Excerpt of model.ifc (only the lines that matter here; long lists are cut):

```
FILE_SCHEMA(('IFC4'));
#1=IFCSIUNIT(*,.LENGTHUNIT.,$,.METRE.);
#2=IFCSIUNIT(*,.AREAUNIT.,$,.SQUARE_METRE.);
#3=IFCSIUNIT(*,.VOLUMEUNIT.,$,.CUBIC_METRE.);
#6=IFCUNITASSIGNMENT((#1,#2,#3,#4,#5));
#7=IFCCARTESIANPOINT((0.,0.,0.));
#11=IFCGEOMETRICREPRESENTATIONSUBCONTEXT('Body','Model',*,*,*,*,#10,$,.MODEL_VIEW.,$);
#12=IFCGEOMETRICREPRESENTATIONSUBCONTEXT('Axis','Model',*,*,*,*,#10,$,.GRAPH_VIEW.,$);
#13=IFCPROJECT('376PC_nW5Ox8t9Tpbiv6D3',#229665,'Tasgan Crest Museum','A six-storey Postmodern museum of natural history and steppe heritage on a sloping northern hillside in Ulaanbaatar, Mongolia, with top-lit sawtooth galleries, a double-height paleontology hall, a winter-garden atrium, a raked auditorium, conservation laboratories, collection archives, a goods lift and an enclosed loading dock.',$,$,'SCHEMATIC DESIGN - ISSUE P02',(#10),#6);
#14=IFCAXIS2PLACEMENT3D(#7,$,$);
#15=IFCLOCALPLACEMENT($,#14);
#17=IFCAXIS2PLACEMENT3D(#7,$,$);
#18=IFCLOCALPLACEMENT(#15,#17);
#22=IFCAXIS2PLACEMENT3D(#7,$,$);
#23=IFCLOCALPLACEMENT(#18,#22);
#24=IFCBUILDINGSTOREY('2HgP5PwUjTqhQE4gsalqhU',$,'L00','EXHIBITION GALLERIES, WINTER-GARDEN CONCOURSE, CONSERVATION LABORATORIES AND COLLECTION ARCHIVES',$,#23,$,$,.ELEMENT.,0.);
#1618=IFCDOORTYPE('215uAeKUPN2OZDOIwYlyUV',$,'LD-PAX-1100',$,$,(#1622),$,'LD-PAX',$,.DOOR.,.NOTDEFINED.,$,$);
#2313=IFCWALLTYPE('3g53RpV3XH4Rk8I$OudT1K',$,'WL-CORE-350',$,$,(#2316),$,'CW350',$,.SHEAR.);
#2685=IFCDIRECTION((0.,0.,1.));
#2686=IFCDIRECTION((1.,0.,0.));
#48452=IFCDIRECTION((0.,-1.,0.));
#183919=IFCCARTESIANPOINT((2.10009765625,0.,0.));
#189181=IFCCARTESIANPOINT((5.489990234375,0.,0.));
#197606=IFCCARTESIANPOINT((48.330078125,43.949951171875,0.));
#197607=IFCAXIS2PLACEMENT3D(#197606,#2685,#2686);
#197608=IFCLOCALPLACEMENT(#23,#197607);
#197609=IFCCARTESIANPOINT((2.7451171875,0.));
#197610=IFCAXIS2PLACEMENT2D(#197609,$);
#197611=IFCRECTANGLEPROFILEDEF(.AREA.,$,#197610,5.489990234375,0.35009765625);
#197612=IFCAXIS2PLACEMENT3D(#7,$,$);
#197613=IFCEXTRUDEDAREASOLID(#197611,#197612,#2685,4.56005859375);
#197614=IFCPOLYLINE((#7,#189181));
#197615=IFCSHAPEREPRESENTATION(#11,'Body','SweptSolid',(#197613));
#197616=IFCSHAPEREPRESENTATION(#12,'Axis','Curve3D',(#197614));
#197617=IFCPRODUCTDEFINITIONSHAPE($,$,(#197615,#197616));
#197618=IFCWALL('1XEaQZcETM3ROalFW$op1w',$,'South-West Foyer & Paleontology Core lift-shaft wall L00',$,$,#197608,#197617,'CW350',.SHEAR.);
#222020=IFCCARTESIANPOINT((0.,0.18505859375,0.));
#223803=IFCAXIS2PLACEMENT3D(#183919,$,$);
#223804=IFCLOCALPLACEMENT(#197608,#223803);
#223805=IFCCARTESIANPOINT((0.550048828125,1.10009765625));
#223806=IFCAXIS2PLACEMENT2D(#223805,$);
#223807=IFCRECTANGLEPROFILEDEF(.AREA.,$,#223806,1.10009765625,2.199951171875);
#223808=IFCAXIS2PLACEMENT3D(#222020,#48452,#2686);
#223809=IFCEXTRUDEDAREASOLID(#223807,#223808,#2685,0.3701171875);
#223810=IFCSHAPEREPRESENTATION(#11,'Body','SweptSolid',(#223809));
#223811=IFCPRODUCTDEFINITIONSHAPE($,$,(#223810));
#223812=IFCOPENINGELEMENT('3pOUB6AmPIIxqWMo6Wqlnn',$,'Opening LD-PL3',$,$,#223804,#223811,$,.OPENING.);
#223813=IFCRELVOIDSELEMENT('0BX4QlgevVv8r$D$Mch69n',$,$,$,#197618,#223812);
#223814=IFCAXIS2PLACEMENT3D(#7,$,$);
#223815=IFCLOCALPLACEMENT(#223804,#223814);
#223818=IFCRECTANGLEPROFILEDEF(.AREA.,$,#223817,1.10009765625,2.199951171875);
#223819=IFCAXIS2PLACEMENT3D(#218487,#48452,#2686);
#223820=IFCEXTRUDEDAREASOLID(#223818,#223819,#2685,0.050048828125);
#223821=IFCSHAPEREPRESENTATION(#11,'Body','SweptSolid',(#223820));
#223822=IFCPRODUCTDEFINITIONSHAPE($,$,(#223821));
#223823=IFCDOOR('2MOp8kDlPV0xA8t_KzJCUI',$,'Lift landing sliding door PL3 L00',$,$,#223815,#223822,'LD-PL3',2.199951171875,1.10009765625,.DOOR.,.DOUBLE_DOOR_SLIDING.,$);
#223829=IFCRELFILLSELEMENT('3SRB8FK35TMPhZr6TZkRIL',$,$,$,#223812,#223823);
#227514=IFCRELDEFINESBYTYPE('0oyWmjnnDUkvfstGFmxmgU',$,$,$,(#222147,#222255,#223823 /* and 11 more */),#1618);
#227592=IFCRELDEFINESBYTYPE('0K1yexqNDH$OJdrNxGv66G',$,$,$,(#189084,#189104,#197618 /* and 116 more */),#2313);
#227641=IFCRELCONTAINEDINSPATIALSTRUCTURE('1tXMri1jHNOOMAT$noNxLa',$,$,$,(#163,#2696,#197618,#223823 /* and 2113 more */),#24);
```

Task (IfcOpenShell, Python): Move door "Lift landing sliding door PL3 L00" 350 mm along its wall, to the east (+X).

```python
import ifcopenshell
import ifcopenshell.api.geometry
import ifcopenshell.util.placement

model = ifcopenshell.open("model.ifc")

door = model.by_guid("2MOp8kDlPV0xA8t_KzJCUI")
opening = door.FillsVoids[0].RelatingOpeningElement
wall = opening.VoidsElements[0].RelatingBuildingElement

wall_matrix = ifcopenshell.util.placement.get_local_placement(wall.ObjectPlacement)
shift = wall_matrix[:3, 0] * 0.35
before = ifcopenshell.util.placement.get_local_placement(door.ObjectPlacement)[:3, 3].copy()

# The door is placed relative to its opening, so it follows when the opening moves.
matrix = ifcopenshell.util.placement.get_local_placement(opening.ObjectPlacement)
matrix[:3, 3] += shift
ifcopenshell.api.geometry.edit_object_placement(
    model, product=opening, matrix=matrix, is_si=False, should_transform_children=True
)

after = ifcopenshell.util.placement.get_local_placement(door.ObjectPlacement)[:3, 3]
print("door moved by", (after - before).round(3) + 0.0)

model.write("model_rev.ifc")
```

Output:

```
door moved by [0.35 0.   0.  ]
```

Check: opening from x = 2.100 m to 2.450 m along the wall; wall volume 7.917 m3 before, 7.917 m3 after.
